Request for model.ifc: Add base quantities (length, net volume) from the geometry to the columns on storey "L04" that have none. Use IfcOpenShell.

First a look at what the model holds.

```python
import ifcopenshell
import ifcopenshell.util.element
import ifcopenshell.util.unit

model = ifcopenshell.open("model.ifc")
print(model.schema)
for unit_type in ("LENGTHUNIT", "AREAUNIT", "VOLUMEUNIT"):
    print(unit_type, ifcopenshell.util.unit.calculate_unit_scale(model, unit_type))
storey = next(s for s in model.by_type("IfcBuildingStorey") if s.Name == "L04")
columns = [e for e in ifcopenshell.util.element.get_decomposition(storey) if e.is_a("IfcColumn")]
for e in sorted(columns, key=lambda e: e.id()):
    print(e.id(), e.is_a(), e.Name, list(ifcopenshell.util.element.get_psets(e, qtos_only=True)), sep=" | ")
```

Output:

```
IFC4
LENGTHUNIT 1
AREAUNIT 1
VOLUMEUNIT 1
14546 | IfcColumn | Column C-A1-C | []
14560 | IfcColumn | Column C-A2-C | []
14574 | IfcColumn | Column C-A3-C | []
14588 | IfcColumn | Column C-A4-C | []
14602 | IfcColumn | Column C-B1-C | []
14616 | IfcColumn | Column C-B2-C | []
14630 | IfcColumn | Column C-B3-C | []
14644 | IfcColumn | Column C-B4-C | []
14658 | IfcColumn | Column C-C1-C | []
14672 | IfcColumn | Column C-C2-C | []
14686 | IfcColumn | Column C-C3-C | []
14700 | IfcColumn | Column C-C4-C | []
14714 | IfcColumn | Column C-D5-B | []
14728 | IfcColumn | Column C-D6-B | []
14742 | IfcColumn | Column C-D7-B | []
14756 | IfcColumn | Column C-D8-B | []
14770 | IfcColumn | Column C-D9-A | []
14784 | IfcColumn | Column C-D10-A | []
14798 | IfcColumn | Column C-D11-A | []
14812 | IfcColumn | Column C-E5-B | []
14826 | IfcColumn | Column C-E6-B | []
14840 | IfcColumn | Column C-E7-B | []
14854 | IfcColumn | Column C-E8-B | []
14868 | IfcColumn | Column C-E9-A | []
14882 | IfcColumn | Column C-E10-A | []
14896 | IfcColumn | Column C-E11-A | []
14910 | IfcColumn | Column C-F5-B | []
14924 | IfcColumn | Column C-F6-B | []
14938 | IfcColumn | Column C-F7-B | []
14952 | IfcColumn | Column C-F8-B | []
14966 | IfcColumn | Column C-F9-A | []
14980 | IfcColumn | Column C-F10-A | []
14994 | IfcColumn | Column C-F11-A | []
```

```python
import ifcopenshell
import ifcopenshell.api.pset
import ifcopenshell.geom
import ifcopenshell.util.element
import ifcopenshell.util.shape
import ifcopenshell.util.unit

model = ifcopenshell.open("model.ifc")
unit_scale = ifcopenshell.util.unit.calculate_unit_scale(model)
volume_scale = ifcopenshell.util.unit.calculate_unit_scale(model, "VOLUMEUNIT")
settings = ifcopenshell.geom.settings()

storey = next(s for s in model.by_type("IfcBuildingStorey") if s.Name == "L04")
columns = [e for e in ifcopenshell.util.element.get_decomposition(storey) if e.is_a("IfcColumn")]

for e in sorted(columns, key=lambda e: e.id()):
    if ifcopenshell.util.element.get_psets(e, qtos_only=True, should_inherit=False):
        continue
    # Geometry comes back in metres, in the element's own axes.
    shape = ifcopenshell.geom.create_shape(settings, e)
    values = {
        "Length": ifcopenshell.util.shape.get_z(shape.geometry) / unit_scale,
        "NetVolume": ifcopenshell.util.shape.get_volume(shape.geometry) / volume_scale,
    }
    qto = ifcopenshell.api.pset.add_qto(model, product=e, name="Qto_ColumnBaseQuantities")
    ifcopenshell.api.pset.edit_qto(model, qto=qto, properties=values)
    print(e.id(), {k: round(v, 3) for k, v in values.items()})

model.write("model_v2.ifc")
```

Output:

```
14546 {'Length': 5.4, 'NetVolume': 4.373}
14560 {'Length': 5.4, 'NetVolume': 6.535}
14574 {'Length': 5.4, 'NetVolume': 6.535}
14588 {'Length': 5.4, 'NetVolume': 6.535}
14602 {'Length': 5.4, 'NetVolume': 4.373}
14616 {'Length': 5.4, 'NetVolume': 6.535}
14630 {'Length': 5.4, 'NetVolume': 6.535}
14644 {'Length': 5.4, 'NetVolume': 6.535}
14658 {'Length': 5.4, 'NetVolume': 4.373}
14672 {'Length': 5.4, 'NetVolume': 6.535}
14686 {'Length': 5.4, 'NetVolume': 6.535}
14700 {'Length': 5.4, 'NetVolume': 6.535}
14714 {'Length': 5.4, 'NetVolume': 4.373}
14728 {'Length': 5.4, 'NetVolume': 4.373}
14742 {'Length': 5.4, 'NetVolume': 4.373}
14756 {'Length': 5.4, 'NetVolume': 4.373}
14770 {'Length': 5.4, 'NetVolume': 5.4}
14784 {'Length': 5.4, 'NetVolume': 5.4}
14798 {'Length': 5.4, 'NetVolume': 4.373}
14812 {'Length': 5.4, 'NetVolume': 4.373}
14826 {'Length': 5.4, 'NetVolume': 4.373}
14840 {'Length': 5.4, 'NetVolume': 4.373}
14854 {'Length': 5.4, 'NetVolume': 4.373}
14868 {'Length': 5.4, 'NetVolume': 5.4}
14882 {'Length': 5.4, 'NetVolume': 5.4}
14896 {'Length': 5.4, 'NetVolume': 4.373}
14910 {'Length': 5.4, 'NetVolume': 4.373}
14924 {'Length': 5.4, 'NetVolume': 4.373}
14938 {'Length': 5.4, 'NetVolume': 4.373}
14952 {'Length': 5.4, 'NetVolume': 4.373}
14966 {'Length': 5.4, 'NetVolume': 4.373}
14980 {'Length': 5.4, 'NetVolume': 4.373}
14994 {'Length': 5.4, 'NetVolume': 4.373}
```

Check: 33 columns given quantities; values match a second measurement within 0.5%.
